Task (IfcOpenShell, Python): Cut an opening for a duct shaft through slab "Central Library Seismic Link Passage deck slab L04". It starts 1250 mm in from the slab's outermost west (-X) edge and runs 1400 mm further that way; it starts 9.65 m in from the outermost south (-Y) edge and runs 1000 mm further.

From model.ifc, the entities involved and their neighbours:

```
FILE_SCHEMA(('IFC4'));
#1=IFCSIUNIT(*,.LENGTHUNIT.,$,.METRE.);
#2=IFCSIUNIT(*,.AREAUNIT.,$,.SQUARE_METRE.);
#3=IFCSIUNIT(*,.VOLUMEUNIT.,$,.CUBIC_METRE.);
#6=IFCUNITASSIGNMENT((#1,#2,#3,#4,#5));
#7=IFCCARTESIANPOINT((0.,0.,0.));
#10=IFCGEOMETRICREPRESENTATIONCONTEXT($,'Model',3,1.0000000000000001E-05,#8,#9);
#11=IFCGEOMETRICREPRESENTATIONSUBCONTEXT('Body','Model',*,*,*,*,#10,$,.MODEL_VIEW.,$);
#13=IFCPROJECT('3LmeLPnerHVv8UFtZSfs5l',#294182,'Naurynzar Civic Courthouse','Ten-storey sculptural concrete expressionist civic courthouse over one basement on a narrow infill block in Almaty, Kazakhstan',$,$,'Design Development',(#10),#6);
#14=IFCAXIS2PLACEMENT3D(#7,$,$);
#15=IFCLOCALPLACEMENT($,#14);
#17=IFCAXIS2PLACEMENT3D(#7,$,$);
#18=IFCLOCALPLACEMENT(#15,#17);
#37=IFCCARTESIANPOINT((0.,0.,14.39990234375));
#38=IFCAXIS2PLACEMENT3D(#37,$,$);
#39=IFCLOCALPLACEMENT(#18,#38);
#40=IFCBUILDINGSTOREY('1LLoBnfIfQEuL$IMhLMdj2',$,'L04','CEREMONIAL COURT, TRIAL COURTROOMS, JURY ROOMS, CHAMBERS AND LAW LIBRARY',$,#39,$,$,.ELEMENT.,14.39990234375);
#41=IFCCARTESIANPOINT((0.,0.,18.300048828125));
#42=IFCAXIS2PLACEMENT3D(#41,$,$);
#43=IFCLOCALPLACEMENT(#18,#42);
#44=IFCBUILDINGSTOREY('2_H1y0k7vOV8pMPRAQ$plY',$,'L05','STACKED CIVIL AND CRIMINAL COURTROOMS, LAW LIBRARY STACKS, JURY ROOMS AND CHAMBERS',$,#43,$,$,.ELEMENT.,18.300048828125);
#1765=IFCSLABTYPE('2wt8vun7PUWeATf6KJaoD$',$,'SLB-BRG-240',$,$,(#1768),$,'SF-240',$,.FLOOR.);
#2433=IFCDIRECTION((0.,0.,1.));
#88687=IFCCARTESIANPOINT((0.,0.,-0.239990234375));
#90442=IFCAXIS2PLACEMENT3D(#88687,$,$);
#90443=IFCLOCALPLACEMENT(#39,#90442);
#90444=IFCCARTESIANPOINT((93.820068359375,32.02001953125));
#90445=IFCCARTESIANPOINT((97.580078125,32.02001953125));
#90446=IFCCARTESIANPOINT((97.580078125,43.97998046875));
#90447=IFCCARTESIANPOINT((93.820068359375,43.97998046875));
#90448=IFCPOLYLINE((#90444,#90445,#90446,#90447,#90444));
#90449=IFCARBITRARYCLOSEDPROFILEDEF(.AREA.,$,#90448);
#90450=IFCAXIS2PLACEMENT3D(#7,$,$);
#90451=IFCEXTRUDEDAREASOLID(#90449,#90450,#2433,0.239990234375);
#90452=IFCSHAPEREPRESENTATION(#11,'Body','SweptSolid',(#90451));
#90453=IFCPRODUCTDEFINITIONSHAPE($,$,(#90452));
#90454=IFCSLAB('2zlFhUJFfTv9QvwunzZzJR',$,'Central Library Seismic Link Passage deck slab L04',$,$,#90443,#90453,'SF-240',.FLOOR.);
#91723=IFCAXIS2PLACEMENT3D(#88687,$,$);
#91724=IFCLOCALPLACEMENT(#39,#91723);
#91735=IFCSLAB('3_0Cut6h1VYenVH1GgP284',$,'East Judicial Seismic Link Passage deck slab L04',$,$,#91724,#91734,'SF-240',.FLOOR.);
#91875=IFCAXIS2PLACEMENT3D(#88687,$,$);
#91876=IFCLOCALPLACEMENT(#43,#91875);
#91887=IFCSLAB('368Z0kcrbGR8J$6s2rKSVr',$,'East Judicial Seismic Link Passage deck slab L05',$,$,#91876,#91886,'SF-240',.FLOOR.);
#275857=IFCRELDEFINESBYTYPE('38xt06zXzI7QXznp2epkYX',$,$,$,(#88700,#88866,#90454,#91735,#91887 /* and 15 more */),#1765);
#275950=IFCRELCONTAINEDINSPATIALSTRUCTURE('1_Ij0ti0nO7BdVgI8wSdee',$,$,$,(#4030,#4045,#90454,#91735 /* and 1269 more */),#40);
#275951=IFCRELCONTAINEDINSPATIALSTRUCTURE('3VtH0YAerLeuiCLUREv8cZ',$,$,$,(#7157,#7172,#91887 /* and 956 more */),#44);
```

```python
import numpy as np
import ifcopenshell
import ifcopenshell.api.feature
import ifcopenshell.api.geometry
import ifcopenshell.api.root
import ifcopenshell.geom
import ifcopenshell.util.placement
import ifcopenshell.util.representation
import ifcopenshell.util.shape
import ifcopenshell.util.unit

model = ifcopenshell.open("model.ifc")
unit_scale = ifcopenshell.util.unit.calculate_unit_scale(model)
settings = ifcopenshell.geom.settings()


def volume(element):
    """Net volume in cubic metres, openings subtracted."""
    shape = ifcopenshell.geom.create_shape(settings, element)
    return ifcopenshell.util.shape.get_volume(shape.geometry)


slab = model.by_id(90454)
before = volume(slab)

# Extent in the slab's own axes, in metres. The edges named are its -X and -Y sides.
slab_shape = ifcopenshell.geom.create_shape(settings, slab)
vertices = ifcopenshell.util.shape.get_vertices(slab_shape.geometry)
x_min, y_min, bottom = vertices.min(axis=0)
top = vertices[:, 2].max()

opening = ifcopenshell.api.root.create_entity(model, ifc_class="IfcOpeningElement", name="Duct shaft opening", predefined_type="OPENING")
context = ifcopenshell.util.representation.get_context(model, "Model", "Body", "MODEL_VIEW")
width, depth = 1.4, 1
outline = [(0.0, 0.0), (width, 0.0), (width, depth), (0.0, depth), (0.0, 0.0)]
# Overshoot both faces by 50 mm so the cut is clean.
shape = ifcopenshell.api.geometry.add_slab_representation(
    model, context=context, depth=top - bottom + 0.1, polyline=outline
)
ifcopenshell.api.geometry.assign_representation(model, product=opening, representation=shape)

matrix = ifcopenshell.util.placement.get_local_placement(slab.ObjectPlacement)
matrix[:, 3] = matrix @ np.append(np.array([x_min + 1.25, y_min + 9.65, bottom - 0.05]) / unit_scale, 1.0)
ifcopenshell.api.geometry.edit_object_placement(model, product=opening, matrix=matrix, is_si=False)
ifcopenshell.api.feature.add_feature(model, feature=opening, element=slab)

after = volume(slab)

print(f"slab volume {before:.3f} -> {after:.3f} m3")

model.write("model_edited.ifc")
```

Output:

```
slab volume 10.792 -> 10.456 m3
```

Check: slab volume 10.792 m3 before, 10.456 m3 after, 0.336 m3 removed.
